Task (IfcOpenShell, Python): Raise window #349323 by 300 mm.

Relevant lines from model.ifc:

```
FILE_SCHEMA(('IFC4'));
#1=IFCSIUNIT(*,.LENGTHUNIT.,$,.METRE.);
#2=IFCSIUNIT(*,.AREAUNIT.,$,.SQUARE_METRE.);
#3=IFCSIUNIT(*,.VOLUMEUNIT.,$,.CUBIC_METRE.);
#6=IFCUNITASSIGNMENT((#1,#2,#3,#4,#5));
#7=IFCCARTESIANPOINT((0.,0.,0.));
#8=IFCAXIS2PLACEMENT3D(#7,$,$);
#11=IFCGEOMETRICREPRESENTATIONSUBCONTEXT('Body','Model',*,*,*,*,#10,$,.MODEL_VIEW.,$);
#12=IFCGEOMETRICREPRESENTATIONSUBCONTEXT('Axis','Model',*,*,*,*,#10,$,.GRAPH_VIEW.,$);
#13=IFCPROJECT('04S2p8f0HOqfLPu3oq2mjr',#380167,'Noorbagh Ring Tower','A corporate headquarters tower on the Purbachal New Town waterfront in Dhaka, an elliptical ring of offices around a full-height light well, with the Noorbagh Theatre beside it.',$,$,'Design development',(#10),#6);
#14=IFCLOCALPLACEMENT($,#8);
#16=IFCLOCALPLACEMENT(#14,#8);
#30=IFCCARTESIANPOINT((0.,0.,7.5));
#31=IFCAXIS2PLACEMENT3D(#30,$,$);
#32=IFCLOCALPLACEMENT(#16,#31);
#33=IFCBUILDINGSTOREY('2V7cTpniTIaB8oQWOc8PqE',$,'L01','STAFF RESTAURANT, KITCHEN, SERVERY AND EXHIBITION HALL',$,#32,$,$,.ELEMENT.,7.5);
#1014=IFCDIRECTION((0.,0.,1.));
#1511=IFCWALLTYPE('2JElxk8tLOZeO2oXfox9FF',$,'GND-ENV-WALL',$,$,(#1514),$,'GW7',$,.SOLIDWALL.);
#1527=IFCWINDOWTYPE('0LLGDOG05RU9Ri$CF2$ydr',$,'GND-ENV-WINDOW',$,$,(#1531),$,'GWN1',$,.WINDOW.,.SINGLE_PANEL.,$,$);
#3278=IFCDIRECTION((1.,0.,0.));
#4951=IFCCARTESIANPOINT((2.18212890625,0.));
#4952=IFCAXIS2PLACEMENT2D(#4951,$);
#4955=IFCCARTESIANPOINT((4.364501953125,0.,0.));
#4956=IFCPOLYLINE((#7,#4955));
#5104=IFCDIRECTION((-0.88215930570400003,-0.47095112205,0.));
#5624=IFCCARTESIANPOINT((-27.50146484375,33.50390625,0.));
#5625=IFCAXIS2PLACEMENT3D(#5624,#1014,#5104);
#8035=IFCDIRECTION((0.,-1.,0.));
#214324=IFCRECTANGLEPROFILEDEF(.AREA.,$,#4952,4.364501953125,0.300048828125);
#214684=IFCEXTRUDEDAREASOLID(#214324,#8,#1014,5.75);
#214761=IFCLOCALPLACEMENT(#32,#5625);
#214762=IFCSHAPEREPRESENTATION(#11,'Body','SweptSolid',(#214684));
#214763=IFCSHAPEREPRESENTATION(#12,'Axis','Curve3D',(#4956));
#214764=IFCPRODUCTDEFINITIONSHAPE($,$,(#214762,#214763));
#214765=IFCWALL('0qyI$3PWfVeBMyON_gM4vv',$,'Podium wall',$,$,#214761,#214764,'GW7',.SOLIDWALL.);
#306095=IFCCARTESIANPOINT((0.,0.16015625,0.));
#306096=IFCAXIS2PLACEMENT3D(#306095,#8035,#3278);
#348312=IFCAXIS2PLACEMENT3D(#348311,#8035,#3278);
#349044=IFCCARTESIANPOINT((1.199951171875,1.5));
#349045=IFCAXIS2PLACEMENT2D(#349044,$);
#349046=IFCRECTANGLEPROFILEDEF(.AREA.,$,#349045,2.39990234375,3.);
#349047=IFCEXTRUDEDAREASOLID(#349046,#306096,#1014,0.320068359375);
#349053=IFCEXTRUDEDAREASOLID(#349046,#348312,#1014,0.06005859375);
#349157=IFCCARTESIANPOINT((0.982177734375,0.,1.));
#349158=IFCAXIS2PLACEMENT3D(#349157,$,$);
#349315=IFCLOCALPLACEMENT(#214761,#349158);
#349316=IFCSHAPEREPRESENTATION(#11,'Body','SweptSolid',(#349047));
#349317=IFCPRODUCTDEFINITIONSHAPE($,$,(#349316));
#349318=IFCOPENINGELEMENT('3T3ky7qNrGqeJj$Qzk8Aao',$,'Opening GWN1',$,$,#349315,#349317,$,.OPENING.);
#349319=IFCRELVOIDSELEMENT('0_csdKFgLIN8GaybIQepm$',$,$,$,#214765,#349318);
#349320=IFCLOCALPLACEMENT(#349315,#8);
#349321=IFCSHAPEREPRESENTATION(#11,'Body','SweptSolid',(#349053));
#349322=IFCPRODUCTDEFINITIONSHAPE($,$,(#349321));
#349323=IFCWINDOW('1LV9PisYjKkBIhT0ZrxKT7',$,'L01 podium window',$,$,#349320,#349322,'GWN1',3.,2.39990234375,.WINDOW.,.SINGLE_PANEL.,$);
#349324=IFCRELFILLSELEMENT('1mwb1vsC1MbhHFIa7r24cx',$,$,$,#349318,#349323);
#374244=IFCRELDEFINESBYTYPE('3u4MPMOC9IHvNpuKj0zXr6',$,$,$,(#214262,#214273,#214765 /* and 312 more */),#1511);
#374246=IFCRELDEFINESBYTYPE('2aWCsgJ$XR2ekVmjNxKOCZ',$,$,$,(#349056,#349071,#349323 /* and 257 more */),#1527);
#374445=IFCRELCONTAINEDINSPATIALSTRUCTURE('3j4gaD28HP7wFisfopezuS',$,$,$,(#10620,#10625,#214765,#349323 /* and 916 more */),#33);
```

```python
import numpy as np
import ifcopenshell
import ifcopenshell.api.geometry
import ifcopenshell.util.placement
import ifcopenshell.util.unit

model = ifcopenshell.open("model.ifc")
unit_scale = ifcopenshell.util.unit.calculate_unit_scale(model)

window = model.by_guid("1LV9PisYjKkBIhT0ZrxKT7")
opening = window.FillsVoids[0].RelatingOpeningElement
dz = 0.3

shift = np.array([0.0, 0.0, dz])
# The window is placed relative to its opening, so it follows when the opening moves.
matrix = ifcopenshell.util.placement.get_local_placement(opening.ObjectPlacement)
matrix[:3, 3] += shift
ifcopenshell.api.geometry.edit_object_placement(
    model, product=opening, matrix=matrix, is_si=False, should_transform_children=True
)

print(f"moved by {dz * unit_scale:+.3f} m")

model.write("model-out.ifc")
```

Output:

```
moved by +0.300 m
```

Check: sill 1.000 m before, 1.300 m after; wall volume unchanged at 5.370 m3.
